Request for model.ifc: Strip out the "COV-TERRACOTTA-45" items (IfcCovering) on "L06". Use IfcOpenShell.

First a look at what the model holds.

```python
import ifcopenshell
import ifcopenshell.util.element

model = ifcopenshell.open("model.ifc")
print(model.schema)
storey = next(s for s in model.by_type("IfcBuildingStorey") if s.Name == "L06")
coverings = [e for e in ifcopenshell.util.element.get_decomposition(storey) if e.is_a("IfcCovering")]
seen = {}
for e in coverings:
    element_type = ifcopenshell.util.element.get_type(e)
    name = element_type.Name if element_type not in (None, e) else None
    seen[name] = seen.get(name, 0) + 1
for name, count in sorted(seen.items(), key=str):
    print(count, "x", name)
```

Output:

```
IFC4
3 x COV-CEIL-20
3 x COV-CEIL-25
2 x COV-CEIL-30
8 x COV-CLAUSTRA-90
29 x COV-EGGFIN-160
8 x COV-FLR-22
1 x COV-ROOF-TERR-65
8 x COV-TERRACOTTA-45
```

```python
import ifcopenshell
import ifcopenshell.api.root
import ifcopenshell.util.element

model = ifcopenshell.open("model.ifc")

storey = next(s for s in model.by_type("IfcBuildingStorey") if s.Name == "L06")
coverings = [e for e in ifcopenshell.util.element.get_decomposition(storey) if e.is_a("IfcCovering")]
targets = [e for e in coverings if (t := ifcopenshell.util.element.get_type(e)) not in (None, e) and t.Name == "COV-TERRACOTTA-45"]

for e in targets:
    ifcopenshell.api.root.remove_product(model, product=e)
print(len(targets), "removed")

model.write("model_edited.ifc")
```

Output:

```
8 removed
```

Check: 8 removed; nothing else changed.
